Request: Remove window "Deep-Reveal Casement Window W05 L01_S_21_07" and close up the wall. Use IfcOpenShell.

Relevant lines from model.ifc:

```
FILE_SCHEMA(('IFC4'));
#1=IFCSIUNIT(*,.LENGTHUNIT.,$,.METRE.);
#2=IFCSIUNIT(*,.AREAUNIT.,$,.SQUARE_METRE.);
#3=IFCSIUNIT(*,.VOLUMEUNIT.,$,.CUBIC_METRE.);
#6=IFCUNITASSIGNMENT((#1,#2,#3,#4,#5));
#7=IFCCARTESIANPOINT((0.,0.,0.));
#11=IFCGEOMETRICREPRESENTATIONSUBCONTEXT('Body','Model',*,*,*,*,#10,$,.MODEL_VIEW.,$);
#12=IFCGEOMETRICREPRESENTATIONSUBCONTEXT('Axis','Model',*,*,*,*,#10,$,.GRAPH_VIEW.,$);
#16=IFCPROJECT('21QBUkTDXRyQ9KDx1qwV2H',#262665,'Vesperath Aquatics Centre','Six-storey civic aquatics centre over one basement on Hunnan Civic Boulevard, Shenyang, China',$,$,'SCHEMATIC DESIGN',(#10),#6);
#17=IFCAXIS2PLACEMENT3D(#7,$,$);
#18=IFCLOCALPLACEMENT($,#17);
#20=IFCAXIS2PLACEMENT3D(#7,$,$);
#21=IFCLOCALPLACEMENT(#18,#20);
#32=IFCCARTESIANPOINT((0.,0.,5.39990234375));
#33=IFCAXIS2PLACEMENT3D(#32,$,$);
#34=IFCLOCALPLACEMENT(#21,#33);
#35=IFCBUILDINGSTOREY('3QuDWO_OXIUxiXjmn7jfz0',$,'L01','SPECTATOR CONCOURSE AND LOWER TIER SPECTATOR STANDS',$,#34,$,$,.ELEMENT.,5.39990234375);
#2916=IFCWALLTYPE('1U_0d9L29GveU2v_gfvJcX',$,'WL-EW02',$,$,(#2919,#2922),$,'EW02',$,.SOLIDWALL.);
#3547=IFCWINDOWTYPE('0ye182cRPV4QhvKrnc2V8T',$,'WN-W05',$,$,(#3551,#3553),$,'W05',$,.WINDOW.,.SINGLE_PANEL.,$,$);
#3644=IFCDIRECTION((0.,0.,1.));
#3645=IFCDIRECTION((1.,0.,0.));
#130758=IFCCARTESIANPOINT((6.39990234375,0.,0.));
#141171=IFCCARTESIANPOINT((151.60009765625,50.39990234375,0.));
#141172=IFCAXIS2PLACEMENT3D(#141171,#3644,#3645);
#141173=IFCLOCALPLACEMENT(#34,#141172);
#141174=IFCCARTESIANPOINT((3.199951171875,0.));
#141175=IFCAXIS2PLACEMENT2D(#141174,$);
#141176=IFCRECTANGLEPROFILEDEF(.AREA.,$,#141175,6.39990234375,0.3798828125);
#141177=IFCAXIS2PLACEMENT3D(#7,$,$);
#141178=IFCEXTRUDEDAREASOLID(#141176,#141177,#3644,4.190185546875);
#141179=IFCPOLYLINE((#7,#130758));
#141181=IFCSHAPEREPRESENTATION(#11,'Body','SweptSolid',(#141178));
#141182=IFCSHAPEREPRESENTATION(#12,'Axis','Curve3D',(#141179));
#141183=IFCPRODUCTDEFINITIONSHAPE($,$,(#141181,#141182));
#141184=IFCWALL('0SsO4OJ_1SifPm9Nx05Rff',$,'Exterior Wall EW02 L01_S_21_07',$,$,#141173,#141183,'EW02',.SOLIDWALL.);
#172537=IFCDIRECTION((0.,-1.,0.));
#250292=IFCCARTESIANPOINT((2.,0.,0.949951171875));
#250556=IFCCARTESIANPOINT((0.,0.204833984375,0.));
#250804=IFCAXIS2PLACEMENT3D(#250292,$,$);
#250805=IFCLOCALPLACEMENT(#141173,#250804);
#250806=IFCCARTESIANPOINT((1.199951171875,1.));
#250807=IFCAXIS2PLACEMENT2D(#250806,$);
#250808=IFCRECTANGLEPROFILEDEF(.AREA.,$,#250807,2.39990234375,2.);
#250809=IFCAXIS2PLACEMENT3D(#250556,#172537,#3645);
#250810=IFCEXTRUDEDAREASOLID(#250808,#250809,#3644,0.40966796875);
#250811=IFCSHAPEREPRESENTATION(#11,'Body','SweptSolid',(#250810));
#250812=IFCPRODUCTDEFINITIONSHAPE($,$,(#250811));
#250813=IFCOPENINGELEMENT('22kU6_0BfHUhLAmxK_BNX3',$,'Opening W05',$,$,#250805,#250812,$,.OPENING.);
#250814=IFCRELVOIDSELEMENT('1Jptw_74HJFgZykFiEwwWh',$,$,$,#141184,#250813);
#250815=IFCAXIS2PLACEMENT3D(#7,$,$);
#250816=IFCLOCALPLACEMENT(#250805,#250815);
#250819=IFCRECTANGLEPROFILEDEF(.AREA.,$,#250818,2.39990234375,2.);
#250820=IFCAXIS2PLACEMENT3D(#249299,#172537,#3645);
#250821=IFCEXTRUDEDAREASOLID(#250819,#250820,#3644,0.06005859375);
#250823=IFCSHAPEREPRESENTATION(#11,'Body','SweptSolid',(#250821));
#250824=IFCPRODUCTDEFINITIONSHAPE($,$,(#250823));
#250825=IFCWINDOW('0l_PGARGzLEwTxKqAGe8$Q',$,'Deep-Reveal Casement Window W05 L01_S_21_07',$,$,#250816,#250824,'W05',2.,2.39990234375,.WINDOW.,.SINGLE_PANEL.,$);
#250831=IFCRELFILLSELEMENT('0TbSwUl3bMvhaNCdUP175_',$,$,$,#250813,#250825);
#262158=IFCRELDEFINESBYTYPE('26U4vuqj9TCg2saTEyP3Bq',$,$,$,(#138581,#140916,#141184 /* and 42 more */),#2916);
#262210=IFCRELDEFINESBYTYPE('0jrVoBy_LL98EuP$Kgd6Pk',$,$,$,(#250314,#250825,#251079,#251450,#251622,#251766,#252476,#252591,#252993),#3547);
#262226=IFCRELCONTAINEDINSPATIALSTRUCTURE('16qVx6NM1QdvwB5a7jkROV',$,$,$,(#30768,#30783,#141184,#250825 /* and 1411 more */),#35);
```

```python
import ifcopenshell
import ifcopenshell.api.feature
import ifcopenshell.api.root
import ifcopenshell.geom
import ifcopenshell.util.shape

model = ifcopenshell.open("model.ifc")
settings = ifcopenshell.geom.settings()


def volume(element):
    """Net volume in cubic metres, openings subtracted."""
    shape = ifcopenshell.geom.create_shape(settings, element)
    return ifcopenshell.util.shape.get_volume(shape.geometry)


window = model.by_guid("0l_PGARGzLEwTxKqAGe8$Q")
opening = window.FillsVoids[0].RelatingOpeningElement
wall = opening.VoidsElements[0].RelatingBuildingElement
before = volume(wall)

ifcopenshell.api.root.remove_product(model, product=window)
ifcopenshell.api.feature.remove_feature(model, feature=opening)

after = volume(wall)

print(f"wall volume {before:.3f} -> {after:.3f} m3")

model.write("model_updated.ifc")
```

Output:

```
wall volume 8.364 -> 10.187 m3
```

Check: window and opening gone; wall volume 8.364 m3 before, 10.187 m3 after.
